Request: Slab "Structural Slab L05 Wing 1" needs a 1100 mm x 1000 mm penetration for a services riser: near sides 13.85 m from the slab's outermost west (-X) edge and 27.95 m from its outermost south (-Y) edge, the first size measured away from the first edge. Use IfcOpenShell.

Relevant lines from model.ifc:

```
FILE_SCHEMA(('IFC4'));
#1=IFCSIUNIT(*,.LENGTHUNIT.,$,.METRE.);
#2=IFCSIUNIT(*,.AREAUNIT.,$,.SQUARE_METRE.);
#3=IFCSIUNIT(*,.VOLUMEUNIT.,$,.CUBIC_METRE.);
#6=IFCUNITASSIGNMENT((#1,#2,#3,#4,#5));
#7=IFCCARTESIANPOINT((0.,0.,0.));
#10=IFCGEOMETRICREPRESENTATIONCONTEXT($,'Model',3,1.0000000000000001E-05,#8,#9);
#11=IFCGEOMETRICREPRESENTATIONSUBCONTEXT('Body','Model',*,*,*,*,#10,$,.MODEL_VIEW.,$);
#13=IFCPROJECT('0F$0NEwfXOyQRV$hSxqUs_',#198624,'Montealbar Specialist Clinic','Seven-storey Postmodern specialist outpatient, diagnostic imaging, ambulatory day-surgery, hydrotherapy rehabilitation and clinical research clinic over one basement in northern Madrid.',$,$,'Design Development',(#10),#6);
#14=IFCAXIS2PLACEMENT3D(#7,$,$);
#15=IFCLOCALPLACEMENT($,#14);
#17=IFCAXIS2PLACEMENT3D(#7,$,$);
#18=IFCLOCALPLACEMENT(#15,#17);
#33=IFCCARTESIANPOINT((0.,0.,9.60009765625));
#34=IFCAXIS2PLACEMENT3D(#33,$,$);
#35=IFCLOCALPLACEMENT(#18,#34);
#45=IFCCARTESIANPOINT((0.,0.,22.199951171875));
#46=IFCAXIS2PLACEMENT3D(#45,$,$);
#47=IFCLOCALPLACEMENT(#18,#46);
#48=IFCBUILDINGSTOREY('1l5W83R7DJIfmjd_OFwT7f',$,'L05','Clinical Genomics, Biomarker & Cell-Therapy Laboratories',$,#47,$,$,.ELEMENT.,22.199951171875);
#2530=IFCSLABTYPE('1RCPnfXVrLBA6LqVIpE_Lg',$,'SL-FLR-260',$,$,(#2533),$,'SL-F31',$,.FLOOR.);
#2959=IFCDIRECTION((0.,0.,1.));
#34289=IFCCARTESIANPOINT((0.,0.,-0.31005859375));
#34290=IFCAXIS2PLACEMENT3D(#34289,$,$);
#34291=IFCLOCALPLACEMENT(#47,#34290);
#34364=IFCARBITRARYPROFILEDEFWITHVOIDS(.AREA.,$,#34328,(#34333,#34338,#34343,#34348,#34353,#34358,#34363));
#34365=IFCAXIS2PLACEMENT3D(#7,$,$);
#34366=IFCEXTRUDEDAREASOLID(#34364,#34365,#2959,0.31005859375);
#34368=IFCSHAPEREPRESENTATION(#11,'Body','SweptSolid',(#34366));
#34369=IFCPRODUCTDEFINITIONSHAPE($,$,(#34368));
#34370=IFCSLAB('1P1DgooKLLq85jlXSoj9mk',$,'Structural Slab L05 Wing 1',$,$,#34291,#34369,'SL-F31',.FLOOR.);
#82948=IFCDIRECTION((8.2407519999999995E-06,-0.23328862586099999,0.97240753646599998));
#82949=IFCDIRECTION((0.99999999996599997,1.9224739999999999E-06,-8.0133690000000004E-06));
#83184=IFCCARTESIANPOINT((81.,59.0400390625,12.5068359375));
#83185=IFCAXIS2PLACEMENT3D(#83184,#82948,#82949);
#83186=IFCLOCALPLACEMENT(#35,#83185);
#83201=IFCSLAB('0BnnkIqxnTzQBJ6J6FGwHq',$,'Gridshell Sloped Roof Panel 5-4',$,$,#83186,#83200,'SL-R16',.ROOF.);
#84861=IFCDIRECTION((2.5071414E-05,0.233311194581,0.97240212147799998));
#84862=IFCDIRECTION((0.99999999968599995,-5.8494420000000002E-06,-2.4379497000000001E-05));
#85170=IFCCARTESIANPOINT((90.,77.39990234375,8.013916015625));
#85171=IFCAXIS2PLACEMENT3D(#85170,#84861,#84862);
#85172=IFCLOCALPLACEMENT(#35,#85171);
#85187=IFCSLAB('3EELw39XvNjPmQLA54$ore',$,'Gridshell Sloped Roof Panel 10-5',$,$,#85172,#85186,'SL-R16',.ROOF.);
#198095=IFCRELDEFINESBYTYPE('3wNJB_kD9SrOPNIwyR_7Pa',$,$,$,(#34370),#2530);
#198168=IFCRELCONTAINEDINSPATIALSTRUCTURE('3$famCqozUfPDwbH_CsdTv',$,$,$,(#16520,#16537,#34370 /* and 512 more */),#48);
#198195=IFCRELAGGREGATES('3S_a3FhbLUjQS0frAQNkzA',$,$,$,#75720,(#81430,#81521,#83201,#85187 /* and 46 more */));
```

```python
import numpy as np
import ifcopenshell
import ifcopenshell.api.feature
import ifcopenshell.api.geometry
import ifcopenshell.api.root
import ifcopenshell.geom
import ifcopenshell.util.placement
import ifcopenshell.util.representation
import ifcopenshell.util.shape
import ifcopenshell.util.unit

model = ifcopenshell.open("model.ifc")
unit_scale = ifcopenshell.util.unit.calculate_unit_scale(model)
settings = ifcopenshell.geom.settings()


def volume(element):
    """Net volume in cubic metres, openings subtracted."""
    shape = ifcopenshell.geom.create_shape(settings, element)
    return ifcopenshell.util.shape.get_volume(shape.geometry)


slab = model.by_guid("1P1DgooKLLq85jlXSoj9mk")
before = volume(slab)

# Extent in the slab's own axes, in metres. The edges named are its -X and -Y sides.
slab_shape = ifcopenshell.geom.create_shape(settings, slab)
vertices = ifcopenshell.util.shape.get_vertices(slab_shape.geometry)
x_min, y_min, bottom = vertices.min(axis=0)
top = vertices[:, 2].max()

opening = ifcopenshell.api.root.create_entity(model, ifc_class="IfcOpeningElement", name="Services riser opening", predefined_type="OPENING")
context = ifcopenshell.util.representation.get_context(model, "Model", "Body", "MODEL_VIEW")
width, depth = 1.1, 1
outline = [(0.0, 0.0), (width, 0.0), (width, depth), (0.0, depth), (0.0, 0.0)]
# Overshoot both faces by 50 mm so the cut is clean.
shape = ifcopenshell.api.geometry.add_slab_representation(
    model, context=context, depth=top - bottom + 0.1, polyline=outline
)
ifcopenshell.api.geometry.assign_representation(model, product=opening, representation=shape)

matrix = ifcopenshell.util.placement.get_local_placement(slab.ObjectPlacement)
matrix[:, 3] = matrix @ np.append(np.array([x_min + 13.85, y_min + 27.95, bottom - 0.05]) / unit_scale, 1.0)
ifcopenshell.api.geometry.edit_object_placement(model, product=opening, matrix=matrix, is_si=False)
ifcopenshell.api.feature.add_feature(model, feature=opening, element=slab)

after = volume(slab)

print(f"slab volume {before:.3f} -> {after:.3f} m3")

model.write("model_updated.ifc")
```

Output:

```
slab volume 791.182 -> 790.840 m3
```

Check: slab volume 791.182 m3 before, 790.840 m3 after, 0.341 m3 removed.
